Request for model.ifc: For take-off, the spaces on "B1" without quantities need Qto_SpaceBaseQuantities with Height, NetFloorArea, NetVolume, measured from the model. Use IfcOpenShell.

First a look at what the model holds.

```python
import ifcopenshell
import ifcopenshell.util.element
import ifcopenshell.util.unit

model = ifcopenshell.open("model.ifc")
print(model.schema)
for unit_type in ("LENGTHUNIT", "AREAUNIT", "VOLUMEUNIT"):
    print(unit_type, ifcopenshell.util.unit.calculate_unit_scale(model, unit_type))
storey = next(s for s in model.by_type("IfcBuildingStorey") if s.Name == "B1")
spaces = [e for e in ifcopenshell.util.element.get_decomposition(storey) if e.is_a("IfcSpace")]
for e in sorted(spaces, key=lambda e: e.id()):
    print(e.id(), e.is_a(), e.Name, list(ifcopenshell.util.element.get_psets(e, qtos_only=True)), sep=" | ")
```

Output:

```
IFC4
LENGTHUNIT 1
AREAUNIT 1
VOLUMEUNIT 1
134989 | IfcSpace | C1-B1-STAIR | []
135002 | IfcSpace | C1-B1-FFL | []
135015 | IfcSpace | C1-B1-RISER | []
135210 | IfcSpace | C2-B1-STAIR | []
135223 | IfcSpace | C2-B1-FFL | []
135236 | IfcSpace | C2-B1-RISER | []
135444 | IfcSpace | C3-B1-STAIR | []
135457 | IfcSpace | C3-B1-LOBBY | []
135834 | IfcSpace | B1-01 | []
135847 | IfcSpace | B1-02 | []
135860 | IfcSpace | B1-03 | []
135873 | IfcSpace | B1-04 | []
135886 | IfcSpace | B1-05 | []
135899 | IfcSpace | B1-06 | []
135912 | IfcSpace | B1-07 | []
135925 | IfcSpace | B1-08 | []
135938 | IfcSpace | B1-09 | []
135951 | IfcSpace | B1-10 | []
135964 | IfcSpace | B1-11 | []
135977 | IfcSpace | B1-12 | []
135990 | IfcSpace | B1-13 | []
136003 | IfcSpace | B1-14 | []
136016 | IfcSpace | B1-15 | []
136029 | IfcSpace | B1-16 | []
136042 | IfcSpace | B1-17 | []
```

```python
import ifcopenshell
import ifcopenshell.api.pset
import ifcopenshell.geom
import ifcopenshell.util.element
import ifcopenshell.util.shape
import ifcopenshell.util.unit

model = ifcopenshell.open("model.ifc")
unit_scale = ifcopenshell.util.unit.calculate_unit_scale(model)
area_scale = ifcopenshell.util.unit.calculate_unit_scale(model, "AREAUNIT")
volume_scale = ifcopenshell.util.unit.calculate_unit_scale(model, "VOLUMEUNIT")
settings = ifcopenshell.geom.settings()

storey = next(s for s in model.by_type("IfcBuildingStorey") if s.Name == "B1")
spaces = [e for e in ifcopenshell.util.element.get_decomposition(storey) if e.is_a("IfcSpace")]

for e in sorted(spaces, key=lambda e: e.id()):
    if ifcopenshell.util.element.get_psets(e, qtos_only=True, should_inherit=False):
        continue
    # Geometry comes back in metres, in the element's own axes.
    shape = ifcopenshell.geom.create_shape(settings, e)
    values = {
        "Height": ifcopenshell.util.shape.get_z(shape.geometry) / unit_scale,
        "NetFloorArea": ifcopenshell.util.shape.get_footprint_area(shape.geometry) / area_scale,
        "NetVolume": ifcopenshell.util.shape.get_volume(shape.geometry) / volume_scale,
    }
    qto = ifcopenshell.api.pset.add_qto(model, product=e, name="Qto_SpaceBaseQuantities")
    ifcopenshell.api.pset.edit_qto(model, qto=qto, properties=values)
    print(e.id(), {k: round(v, 3) for k, v in values.items()})

model.write("model_edited.ifc")
```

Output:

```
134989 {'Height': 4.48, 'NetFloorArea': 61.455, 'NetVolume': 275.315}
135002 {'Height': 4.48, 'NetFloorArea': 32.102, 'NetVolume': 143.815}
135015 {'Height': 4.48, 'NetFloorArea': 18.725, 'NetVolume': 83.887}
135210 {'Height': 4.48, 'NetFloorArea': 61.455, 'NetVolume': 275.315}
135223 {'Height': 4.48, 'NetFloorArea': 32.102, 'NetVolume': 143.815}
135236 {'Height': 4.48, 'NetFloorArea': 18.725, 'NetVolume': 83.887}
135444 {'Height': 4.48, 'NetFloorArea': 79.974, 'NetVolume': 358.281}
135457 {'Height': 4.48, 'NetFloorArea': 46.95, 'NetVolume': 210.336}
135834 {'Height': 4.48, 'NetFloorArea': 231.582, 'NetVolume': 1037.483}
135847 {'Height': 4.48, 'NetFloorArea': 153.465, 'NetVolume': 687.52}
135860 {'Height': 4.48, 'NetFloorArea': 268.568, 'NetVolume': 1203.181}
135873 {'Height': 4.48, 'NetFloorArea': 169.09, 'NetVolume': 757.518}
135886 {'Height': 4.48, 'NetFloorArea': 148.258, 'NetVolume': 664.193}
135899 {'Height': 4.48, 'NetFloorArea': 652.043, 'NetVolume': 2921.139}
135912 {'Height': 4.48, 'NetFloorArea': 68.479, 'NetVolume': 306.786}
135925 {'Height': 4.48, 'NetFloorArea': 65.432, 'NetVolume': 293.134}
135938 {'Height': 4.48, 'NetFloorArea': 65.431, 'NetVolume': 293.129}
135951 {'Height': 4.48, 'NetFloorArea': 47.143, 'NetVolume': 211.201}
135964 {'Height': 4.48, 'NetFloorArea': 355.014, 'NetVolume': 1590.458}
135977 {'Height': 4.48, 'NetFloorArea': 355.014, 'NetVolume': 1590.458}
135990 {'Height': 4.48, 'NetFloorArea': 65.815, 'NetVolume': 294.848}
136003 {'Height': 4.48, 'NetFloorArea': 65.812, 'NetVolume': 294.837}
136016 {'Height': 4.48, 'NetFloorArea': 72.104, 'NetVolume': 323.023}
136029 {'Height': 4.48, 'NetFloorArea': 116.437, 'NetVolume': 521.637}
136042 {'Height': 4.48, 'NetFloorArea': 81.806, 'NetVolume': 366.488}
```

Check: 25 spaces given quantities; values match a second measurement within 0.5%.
